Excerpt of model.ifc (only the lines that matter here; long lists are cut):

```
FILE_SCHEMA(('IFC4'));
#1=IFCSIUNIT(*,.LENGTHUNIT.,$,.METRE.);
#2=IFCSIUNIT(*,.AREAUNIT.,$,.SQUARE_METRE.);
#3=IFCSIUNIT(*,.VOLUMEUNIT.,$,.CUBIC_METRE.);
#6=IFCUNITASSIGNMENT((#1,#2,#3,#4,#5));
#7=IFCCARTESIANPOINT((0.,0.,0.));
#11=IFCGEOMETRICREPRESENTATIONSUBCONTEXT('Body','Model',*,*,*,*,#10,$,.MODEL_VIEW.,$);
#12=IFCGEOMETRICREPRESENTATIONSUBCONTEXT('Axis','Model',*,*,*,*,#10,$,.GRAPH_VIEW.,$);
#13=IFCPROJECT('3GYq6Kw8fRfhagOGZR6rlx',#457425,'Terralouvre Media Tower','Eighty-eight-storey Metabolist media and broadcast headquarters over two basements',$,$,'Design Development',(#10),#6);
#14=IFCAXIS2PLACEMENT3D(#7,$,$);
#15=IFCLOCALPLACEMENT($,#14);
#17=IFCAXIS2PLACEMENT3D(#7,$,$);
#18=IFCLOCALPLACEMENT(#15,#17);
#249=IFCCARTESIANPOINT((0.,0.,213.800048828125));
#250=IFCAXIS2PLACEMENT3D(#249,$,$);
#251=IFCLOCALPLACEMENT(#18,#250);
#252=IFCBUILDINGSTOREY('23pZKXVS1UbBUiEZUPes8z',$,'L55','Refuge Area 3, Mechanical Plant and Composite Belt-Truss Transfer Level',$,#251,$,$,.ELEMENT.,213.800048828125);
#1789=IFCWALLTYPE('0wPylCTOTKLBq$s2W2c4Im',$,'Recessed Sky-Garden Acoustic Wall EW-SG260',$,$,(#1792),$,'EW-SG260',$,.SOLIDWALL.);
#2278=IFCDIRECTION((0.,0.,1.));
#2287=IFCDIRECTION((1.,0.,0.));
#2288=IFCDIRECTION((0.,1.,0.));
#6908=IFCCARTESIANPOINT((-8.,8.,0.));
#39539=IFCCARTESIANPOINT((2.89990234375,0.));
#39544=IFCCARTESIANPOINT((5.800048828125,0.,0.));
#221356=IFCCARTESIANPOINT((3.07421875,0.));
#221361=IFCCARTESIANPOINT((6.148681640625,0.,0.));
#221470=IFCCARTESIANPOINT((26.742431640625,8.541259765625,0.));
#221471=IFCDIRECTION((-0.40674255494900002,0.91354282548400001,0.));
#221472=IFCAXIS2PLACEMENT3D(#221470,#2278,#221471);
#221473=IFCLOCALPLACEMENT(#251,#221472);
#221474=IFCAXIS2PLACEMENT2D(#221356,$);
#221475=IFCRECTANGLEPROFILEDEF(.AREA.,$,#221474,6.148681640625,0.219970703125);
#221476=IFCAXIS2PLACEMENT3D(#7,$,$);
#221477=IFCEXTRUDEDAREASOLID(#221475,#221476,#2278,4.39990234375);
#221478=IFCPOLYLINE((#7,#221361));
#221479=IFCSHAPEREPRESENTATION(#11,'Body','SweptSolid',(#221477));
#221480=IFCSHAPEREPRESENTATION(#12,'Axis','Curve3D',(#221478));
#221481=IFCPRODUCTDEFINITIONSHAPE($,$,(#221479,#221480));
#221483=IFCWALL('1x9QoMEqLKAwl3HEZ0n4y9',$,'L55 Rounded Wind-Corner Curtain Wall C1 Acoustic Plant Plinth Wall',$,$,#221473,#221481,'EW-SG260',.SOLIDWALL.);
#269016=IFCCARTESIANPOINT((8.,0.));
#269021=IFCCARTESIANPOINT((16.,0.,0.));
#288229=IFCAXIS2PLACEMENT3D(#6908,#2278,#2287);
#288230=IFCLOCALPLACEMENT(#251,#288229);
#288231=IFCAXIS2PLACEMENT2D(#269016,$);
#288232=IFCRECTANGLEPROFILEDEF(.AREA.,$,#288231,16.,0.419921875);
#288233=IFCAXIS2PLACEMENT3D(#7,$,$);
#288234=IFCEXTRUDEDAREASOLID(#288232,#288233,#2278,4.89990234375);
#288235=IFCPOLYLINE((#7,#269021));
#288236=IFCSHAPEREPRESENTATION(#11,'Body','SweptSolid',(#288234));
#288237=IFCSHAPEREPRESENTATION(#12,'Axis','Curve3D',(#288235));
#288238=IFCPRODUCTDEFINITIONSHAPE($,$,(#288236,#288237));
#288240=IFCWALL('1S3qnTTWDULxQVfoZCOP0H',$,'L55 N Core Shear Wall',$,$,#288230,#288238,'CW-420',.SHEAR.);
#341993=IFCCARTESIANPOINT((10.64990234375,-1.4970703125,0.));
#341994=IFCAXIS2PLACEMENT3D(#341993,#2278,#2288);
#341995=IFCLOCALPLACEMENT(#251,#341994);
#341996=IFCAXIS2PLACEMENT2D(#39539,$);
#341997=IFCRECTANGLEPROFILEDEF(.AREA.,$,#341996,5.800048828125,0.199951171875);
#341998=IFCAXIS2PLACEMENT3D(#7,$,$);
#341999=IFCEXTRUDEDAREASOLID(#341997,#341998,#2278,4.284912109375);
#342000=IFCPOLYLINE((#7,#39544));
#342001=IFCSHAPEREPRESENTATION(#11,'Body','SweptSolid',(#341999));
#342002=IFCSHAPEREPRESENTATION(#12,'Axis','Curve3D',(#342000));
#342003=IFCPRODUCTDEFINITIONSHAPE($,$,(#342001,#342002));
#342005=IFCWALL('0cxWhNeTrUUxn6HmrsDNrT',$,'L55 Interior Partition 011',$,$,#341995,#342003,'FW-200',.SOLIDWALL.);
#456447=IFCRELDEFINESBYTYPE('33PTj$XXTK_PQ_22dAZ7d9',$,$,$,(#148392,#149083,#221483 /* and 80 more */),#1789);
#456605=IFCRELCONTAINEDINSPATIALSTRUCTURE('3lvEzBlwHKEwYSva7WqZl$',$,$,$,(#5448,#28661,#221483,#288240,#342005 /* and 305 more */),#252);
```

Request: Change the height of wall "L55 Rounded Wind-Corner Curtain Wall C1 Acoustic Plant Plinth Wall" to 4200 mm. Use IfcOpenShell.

```python
import ifcopenshell
import ifcopenshell.geom
import ifcopenshell.util.representation
import ifcopenshell.util.shape

model = ifcopenshell.open("model.ifc")
settings = ifcopenshell.geom.settings()


def volume(element):
    """Net volume in cubic metres, openings subtracted."""
    shape = ifcopenshell.geom.create_shape(settings, element)
    return ifcopenshell.util.shape.get_volume(shape.geometry)


wall = model.by_id(221483)
before = volume(wall)

body = ifcopenshell.util.representation.get_representation(wall, "Model", "Body")
solid = body.Items[0]
old_height = solid.Depth
solid.Depth = 4.2
after = volume(wall)

print(f"height {old_height:g} -> {solid.Depth:g}, volume {before:.3f} -> {after:.3f} m3")

model.write("model-out.ifc")
```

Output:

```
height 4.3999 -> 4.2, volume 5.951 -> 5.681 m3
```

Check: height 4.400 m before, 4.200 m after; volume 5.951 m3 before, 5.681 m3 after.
